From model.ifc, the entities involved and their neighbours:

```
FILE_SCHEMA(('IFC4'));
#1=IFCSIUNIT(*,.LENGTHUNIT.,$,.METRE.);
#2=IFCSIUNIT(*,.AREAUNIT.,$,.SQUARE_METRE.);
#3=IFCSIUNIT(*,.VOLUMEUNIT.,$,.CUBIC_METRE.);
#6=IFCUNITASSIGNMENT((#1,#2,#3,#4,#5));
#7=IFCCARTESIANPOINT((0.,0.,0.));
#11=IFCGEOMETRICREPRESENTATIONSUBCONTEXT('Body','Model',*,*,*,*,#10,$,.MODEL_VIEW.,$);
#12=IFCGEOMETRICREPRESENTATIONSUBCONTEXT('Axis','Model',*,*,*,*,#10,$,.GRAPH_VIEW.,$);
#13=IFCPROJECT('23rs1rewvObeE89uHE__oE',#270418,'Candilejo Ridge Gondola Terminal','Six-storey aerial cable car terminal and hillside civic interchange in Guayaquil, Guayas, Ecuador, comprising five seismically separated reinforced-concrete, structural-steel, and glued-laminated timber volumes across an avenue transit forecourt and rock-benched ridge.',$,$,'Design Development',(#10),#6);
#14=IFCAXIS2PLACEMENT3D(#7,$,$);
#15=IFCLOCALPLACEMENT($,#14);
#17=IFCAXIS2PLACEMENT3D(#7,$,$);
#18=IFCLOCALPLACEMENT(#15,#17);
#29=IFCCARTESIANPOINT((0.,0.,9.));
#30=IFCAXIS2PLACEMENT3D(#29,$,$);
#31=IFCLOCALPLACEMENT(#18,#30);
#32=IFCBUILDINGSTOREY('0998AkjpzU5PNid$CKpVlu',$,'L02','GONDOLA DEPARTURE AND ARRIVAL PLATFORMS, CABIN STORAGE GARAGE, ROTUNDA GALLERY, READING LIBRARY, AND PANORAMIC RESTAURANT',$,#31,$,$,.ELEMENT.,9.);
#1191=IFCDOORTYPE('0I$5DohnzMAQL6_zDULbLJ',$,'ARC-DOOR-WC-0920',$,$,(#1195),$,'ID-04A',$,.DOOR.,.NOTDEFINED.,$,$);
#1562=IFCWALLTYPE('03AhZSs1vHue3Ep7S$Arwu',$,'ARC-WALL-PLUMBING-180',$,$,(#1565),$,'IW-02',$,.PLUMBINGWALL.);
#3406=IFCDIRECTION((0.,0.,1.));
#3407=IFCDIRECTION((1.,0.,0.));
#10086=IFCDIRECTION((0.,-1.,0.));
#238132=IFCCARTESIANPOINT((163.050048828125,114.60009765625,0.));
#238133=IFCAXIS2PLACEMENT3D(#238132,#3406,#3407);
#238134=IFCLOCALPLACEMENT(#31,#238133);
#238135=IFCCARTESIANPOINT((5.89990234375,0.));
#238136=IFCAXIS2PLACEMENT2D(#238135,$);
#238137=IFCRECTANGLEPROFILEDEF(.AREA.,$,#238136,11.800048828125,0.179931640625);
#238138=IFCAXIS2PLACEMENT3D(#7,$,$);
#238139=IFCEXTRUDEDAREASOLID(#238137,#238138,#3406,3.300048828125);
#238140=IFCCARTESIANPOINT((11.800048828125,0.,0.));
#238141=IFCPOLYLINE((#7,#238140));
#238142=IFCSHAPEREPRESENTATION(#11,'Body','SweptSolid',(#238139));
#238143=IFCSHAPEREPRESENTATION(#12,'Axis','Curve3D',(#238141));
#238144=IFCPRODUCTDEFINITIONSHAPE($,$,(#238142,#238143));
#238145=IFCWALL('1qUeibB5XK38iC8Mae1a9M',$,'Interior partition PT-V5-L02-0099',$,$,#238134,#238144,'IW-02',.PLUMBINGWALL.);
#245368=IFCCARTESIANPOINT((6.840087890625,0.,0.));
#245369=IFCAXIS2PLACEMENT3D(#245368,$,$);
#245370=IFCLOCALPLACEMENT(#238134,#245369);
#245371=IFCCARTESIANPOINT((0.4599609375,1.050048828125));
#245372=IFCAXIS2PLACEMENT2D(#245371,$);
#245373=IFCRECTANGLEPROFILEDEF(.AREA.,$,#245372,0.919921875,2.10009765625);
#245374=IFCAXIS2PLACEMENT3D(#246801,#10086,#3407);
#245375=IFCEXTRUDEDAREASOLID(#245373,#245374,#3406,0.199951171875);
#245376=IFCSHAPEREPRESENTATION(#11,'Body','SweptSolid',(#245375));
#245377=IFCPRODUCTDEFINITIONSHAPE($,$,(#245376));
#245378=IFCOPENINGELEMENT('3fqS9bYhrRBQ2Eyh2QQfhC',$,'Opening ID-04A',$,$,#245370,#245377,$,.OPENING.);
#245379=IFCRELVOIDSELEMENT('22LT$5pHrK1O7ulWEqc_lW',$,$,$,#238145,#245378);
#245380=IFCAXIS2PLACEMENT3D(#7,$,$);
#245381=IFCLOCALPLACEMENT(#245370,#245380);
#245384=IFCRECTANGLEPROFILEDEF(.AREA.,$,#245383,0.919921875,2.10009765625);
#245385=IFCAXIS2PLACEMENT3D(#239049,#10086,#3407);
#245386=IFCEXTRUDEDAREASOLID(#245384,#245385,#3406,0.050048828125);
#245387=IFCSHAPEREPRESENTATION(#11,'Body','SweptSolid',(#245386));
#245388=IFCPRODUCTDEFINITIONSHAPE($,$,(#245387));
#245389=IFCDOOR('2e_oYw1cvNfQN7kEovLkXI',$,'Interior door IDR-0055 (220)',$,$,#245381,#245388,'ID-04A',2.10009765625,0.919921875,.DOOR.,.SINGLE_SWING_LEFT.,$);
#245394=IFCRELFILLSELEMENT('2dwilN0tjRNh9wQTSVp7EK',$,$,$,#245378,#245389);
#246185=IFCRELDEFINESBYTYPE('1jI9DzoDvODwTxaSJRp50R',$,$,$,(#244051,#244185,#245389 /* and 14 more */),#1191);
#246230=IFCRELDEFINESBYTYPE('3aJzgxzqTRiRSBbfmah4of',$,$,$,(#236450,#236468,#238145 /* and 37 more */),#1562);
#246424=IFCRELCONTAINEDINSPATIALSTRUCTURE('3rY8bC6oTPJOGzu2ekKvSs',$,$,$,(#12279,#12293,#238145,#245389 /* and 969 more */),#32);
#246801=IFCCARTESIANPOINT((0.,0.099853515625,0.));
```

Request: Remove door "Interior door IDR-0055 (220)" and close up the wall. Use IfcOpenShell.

```python
import ifcopenshell
import ifcopenshell.api.feature
import ifcopenshell.api.root
import ifcopenshell.geom
import ifcopenshell.util.shape

model = ifcopenshell.open("model.ifc")
settings = ifcopenshell.geom.settings()


def volume(element):
    """Net volume in cubic metres, openings subtracted."""
    shape = ifcopenshell.geom.create_shape(settings, element)
    return ifcopenshell.util.shape.get_volume(shape.geometry)


door = model.by_guid("2e_oYw1cvNfQN7kEovLkXI")
opening = door.FillsVoids[0].RelatingOpeningElement
wall = opening.VoidsElements[0].RelatingBuildingElement
before = volume(wall)

ifcopenshell.api.root.remove_product(model, product=door)
ifcopenshell.api.feature.remove_feature(model, feature=opening)

after = volume(wall)

print(f"wall volume {before:.3f} -> {after:.3f} m3")

model.write("model-out.ifc")
```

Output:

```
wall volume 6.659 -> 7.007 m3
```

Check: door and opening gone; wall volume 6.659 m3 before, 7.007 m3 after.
